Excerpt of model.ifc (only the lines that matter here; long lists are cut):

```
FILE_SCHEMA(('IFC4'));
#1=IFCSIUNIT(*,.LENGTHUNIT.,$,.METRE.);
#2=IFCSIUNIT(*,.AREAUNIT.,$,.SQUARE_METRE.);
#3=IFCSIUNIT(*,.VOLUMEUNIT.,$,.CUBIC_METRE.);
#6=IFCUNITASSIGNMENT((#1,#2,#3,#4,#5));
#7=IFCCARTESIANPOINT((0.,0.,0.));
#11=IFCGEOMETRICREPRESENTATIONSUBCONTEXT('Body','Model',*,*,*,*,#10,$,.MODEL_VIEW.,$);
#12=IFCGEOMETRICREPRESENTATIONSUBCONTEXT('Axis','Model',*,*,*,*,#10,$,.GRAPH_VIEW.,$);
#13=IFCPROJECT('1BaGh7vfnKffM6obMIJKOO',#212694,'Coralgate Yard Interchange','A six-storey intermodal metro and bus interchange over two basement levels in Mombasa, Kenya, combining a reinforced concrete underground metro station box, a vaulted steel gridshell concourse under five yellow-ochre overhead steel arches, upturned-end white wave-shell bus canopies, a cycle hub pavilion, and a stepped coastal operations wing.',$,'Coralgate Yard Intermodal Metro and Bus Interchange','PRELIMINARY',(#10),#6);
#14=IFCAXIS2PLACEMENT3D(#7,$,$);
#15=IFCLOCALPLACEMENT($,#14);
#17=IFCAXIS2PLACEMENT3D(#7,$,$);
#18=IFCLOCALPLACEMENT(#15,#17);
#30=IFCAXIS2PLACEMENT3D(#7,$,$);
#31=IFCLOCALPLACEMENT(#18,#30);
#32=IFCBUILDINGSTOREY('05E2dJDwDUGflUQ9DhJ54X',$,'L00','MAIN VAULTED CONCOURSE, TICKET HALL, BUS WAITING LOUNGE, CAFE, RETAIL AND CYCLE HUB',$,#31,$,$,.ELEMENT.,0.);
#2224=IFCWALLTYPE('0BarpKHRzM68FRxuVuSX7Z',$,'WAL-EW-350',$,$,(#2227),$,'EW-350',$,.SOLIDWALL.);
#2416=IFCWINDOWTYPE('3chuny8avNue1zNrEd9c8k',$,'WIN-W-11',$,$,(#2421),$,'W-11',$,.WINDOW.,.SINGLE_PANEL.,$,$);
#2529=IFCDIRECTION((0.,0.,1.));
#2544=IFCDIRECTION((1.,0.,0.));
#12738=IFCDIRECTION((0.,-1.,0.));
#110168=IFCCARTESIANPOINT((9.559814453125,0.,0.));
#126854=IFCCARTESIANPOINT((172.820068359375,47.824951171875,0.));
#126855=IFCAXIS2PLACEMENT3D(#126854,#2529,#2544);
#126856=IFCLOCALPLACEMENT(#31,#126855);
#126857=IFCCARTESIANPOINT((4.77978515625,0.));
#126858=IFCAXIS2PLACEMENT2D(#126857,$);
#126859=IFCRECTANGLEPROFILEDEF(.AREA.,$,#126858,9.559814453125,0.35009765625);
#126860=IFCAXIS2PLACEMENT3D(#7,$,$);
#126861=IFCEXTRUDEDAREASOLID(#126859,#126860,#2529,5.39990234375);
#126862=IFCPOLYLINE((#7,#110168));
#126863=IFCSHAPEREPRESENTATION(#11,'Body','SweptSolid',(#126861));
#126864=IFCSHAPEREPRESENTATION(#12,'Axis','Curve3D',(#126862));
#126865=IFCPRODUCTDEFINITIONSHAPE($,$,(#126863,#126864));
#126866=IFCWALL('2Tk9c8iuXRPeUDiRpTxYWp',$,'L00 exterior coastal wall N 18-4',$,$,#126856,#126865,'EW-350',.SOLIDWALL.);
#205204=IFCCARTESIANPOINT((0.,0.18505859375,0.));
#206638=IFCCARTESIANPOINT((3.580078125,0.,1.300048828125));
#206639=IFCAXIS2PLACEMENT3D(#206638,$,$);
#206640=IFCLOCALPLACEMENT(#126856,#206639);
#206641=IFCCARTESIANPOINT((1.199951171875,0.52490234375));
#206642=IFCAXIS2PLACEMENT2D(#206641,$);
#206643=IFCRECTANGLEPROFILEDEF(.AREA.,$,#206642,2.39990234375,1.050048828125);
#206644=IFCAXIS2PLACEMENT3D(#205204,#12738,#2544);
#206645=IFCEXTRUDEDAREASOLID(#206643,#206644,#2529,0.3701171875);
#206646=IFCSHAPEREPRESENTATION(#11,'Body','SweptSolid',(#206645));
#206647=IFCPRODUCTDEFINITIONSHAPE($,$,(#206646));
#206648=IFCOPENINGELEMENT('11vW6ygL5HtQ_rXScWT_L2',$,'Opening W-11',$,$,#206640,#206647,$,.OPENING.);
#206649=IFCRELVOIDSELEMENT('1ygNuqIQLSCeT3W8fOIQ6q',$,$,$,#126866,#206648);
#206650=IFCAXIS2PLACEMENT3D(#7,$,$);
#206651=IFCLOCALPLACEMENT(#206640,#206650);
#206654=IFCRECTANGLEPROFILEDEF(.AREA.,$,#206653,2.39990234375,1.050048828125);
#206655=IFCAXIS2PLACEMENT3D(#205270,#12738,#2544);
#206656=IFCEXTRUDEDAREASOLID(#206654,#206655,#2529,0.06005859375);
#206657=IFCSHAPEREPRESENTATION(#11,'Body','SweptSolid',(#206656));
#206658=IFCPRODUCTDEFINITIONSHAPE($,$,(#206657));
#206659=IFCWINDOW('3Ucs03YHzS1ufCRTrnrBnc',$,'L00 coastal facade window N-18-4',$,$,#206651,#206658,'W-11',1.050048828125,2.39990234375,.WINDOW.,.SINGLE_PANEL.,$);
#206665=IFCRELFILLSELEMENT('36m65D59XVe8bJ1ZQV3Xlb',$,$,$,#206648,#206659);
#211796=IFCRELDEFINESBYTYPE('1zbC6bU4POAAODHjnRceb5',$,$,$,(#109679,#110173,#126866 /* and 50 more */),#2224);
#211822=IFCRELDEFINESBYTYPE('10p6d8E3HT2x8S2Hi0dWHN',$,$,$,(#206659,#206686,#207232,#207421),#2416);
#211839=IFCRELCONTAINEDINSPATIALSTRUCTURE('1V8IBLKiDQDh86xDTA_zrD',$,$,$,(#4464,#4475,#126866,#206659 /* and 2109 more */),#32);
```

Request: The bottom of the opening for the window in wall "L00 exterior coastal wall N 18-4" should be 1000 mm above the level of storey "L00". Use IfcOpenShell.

```python
import numpy as np
import ifcopenshell
import ifcopenshell.api.geometry
import ifcopenshell.geom
import ifcopenshell.util.element
import ifcopenshell.util.placement
import ifcopenshell.util.shape
import ifcopenshell.util.unit

model = ifcopenshell.open("model.ifc")
unit_scale = ifcopenshell.util.unit.calculate_unit_scale(model)

window = model.by_guid("3Ucs03YHzS1ufCRTrnrBnc")
opening = window.FillsVoids[0].RelatingOpeningElement
storey = ifcopenshell.util.element.get_container(window, ifc_class="IfcBuildingStorey")
level = ifcopenshell.util.placement.get_local_placement(storey.ObjectPlacement)[2, 3]

# The opening's origin need not be at the sill, so measure its lowest point.
shape = ifcopenshell.geom.create_shape(ifcopenshell.geom.settings(), opening)
bottom = ifcopenshell.util.shape.get_shape_bottom_elevation(shape, shape.geometry) / unit_scale
dz = level + 1 / unit_scale - bottom

shift = np.array([0.0, 0.0, dz])
# The window is placed relative to its opening, so it follows when the opening moves.
matrix = ifcopenshell.util.placement.get_local_placement(opening.ObjectPlacement)
matrix[:3, 3] += shift
ifcopenshell.api.geometry.edit_object_placement(
    model, product=opening, matrix=matrix, is_si=False, should_transform_children=True
)

print(f"moved by {dz * unit_scale:+.3f} m")

model.write("model-out.ifc")
```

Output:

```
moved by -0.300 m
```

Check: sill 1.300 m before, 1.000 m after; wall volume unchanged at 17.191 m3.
